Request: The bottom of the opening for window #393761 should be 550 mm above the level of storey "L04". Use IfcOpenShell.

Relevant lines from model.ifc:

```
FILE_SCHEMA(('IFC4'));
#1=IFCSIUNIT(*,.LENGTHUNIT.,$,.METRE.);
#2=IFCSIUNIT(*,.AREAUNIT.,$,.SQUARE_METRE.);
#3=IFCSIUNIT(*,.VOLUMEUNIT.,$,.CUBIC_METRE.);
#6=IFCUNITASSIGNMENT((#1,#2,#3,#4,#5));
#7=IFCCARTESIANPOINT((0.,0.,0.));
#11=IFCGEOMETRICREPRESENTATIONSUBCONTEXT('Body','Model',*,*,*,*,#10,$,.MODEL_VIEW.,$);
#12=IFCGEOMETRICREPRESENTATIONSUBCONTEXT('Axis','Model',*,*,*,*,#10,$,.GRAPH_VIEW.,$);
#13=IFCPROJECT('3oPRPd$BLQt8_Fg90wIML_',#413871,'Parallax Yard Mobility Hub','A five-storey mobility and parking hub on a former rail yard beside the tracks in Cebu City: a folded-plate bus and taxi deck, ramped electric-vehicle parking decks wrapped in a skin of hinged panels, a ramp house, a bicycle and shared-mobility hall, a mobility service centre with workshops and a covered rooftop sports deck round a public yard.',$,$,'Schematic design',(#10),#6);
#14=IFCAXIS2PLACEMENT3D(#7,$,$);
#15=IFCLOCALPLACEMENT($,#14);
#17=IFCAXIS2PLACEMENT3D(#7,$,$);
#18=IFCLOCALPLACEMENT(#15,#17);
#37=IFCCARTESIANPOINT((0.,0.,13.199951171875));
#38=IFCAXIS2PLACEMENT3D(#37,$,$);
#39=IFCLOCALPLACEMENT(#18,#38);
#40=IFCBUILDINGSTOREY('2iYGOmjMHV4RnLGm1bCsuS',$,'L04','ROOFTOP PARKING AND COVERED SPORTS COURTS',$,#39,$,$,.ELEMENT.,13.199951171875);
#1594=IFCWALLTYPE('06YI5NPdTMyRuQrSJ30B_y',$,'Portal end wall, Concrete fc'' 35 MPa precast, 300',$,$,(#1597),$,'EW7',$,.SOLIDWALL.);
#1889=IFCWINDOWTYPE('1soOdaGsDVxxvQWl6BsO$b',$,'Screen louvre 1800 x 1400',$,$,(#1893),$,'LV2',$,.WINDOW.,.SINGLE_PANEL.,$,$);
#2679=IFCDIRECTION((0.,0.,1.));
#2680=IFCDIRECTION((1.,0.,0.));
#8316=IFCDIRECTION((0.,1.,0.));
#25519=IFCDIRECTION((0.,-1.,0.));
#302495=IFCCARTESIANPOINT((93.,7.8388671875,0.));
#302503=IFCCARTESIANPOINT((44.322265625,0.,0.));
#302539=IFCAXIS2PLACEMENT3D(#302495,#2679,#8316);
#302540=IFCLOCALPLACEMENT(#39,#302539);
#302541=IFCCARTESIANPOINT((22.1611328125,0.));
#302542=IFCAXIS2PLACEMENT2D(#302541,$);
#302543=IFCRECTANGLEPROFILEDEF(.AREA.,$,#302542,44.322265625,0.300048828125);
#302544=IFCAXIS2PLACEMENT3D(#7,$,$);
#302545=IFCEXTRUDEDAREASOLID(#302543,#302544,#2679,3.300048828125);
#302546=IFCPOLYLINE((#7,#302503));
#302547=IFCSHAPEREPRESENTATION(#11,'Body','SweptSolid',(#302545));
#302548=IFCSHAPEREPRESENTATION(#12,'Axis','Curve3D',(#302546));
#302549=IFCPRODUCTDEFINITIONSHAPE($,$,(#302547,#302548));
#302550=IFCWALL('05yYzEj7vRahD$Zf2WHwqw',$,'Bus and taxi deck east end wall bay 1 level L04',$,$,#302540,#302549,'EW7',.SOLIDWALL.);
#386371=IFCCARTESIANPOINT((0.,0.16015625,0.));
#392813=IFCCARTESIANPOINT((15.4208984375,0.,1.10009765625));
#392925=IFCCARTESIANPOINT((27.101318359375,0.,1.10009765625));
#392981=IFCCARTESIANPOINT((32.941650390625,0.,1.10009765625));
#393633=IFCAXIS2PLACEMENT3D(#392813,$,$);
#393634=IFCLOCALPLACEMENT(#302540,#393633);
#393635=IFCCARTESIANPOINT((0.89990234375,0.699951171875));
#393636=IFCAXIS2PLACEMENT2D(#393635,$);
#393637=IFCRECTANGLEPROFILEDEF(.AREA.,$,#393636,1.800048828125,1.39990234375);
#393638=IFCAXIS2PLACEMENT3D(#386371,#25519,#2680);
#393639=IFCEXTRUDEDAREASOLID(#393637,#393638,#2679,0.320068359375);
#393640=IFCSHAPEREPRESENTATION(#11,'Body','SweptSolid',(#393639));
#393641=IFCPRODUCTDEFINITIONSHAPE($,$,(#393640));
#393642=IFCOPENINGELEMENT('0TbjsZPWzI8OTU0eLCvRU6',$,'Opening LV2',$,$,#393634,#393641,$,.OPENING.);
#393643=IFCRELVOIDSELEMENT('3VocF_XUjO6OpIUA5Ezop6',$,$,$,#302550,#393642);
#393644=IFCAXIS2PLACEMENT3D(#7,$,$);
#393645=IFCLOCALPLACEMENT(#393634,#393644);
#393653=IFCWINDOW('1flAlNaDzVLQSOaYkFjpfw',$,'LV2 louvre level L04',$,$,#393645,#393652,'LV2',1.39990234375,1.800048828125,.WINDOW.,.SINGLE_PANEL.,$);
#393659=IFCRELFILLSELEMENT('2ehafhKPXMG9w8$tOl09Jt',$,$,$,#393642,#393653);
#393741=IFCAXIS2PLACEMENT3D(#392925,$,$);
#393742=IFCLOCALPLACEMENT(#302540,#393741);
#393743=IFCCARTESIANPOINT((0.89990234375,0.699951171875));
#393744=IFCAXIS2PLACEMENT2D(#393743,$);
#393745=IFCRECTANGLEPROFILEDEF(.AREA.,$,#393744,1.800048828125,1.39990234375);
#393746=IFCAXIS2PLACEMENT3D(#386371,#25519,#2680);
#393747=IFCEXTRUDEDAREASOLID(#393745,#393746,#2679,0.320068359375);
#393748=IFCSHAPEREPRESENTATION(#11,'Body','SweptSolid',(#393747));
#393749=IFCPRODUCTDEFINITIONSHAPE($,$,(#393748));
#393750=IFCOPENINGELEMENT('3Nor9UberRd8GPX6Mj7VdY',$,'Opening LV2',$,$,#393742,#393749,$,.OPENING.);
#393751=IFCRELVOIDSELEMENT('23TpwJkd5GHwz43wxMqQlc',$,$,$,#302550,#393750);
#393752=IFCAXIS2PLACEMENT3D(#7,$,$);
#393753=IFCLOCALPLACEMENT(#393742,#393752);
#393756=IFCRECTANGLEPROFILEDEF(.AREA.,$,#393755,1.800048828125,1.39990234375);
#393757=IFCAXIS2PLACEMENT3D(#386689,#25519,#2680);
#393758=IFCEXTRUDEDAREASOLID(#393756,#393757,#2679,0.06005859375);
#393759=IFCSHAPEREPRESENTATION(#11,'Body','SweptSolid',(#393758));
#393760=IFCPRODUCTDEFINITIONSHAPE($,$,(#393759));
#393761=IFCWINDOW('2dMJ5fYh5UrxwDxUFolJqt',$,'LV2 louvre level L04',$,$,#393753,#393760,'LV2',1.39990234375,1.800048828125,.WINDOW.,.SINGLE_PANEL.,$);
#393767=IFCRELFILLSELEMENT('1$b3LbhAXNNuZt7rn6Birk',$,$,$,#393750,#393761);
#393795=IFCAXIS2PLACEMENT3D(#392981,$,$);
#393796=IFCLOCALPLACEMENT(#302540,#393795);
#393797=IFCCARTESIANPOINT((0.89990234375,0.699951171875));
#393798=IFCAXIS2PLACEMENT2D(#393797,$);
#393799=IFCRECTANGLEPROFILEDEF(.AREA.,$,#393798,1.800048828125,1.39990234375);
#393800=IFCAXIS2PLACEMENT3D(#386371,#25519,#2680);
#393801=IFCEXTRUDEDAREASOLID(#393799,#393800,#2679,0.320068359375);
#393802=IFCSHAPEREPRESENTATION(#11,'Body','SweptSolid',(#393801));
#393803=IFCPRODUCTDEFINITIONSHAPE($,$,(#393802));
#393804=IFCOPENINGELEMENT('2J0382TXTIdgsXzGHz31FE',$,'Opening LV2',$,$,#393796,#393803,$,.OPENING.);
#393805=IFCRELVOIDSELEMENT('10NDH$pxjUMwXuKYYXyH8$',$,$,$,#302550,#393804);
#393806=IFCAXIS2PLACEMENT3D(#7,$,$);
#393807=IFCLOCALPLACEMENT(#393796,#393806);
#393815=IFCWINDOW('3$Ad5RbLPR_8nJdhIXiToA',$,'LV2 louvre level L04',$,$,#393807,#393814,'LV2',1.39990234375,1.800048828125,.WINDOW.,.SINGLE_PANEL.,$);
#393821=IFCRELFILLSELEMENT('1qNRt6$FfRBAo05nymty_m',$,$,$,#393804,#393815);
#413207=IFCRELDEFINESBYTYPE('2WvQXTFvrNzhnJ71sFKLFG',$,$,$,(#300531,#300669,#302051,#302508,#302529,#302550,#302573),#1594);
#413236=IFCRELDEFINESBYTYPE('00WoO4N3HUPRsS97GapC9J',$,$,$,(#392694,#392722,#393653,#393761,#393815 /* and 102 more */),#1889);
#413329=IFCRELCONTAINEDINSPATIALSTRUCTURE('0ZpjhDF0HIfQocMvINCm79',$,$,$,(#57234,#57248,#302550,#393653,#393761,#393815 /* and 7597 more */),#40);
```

```python
import numpy as np
import ifcopenshell
import ifcopenshell.api.geometry
import ifcopenshell.geom
import ifcopenshell.util.element
import ifcopenshell.util.placement
import ifcopenshell.util.shape
import ifcopenshell.util.unit

model = ifcopenshell.open("model.ifc")
unit_scale = ifcopenshell.util.unit.calculate_unit_scale(model)

window = model.by_guid("2dMJ5fYh5UrxwDxUFolJqt")
opening = window.FillsVoids[0].RelatingOpeningElement
storey = ifcopenshell.util.element.get_container(window, ifc_class="IfcBuildingStorey")
level = ifcopenshell.util.placement.get_local_placement(storey.ObjectPlacement)[2, 3]

# The opening's origin need not be at the sill, so measure its lowest point.
shape = ifcopenshell.geom.create_shape(ifcopenshell.geom.settings(), opening)
bottom = ifcopenshell.util.shape.get_shape_bottom_elevation(shape, shape.geometry) / unit_scale
dz = level + 0.55 / unit_scale - bottom

shift = np.array([0.0, 0.0, dz])
# The window is placed relative to its opening, so it follows when the opening moves.
matrix = ifcopenshell.util.placement.get_local_placement(opening.ObjectPlacement)
matrix[:3, 3] += shift
ifcopenshell.api.geometry.edit_object_placement(
    model, product=opening, matrix=matrix, is_si=False, should_transform_children=True
)

print(f"moved by {dz * unit_scale:+.3f} m")

model.write("model-out.ifc")
```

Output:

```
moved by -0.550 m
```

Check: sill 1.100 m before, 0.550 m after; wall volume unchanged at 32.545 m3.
